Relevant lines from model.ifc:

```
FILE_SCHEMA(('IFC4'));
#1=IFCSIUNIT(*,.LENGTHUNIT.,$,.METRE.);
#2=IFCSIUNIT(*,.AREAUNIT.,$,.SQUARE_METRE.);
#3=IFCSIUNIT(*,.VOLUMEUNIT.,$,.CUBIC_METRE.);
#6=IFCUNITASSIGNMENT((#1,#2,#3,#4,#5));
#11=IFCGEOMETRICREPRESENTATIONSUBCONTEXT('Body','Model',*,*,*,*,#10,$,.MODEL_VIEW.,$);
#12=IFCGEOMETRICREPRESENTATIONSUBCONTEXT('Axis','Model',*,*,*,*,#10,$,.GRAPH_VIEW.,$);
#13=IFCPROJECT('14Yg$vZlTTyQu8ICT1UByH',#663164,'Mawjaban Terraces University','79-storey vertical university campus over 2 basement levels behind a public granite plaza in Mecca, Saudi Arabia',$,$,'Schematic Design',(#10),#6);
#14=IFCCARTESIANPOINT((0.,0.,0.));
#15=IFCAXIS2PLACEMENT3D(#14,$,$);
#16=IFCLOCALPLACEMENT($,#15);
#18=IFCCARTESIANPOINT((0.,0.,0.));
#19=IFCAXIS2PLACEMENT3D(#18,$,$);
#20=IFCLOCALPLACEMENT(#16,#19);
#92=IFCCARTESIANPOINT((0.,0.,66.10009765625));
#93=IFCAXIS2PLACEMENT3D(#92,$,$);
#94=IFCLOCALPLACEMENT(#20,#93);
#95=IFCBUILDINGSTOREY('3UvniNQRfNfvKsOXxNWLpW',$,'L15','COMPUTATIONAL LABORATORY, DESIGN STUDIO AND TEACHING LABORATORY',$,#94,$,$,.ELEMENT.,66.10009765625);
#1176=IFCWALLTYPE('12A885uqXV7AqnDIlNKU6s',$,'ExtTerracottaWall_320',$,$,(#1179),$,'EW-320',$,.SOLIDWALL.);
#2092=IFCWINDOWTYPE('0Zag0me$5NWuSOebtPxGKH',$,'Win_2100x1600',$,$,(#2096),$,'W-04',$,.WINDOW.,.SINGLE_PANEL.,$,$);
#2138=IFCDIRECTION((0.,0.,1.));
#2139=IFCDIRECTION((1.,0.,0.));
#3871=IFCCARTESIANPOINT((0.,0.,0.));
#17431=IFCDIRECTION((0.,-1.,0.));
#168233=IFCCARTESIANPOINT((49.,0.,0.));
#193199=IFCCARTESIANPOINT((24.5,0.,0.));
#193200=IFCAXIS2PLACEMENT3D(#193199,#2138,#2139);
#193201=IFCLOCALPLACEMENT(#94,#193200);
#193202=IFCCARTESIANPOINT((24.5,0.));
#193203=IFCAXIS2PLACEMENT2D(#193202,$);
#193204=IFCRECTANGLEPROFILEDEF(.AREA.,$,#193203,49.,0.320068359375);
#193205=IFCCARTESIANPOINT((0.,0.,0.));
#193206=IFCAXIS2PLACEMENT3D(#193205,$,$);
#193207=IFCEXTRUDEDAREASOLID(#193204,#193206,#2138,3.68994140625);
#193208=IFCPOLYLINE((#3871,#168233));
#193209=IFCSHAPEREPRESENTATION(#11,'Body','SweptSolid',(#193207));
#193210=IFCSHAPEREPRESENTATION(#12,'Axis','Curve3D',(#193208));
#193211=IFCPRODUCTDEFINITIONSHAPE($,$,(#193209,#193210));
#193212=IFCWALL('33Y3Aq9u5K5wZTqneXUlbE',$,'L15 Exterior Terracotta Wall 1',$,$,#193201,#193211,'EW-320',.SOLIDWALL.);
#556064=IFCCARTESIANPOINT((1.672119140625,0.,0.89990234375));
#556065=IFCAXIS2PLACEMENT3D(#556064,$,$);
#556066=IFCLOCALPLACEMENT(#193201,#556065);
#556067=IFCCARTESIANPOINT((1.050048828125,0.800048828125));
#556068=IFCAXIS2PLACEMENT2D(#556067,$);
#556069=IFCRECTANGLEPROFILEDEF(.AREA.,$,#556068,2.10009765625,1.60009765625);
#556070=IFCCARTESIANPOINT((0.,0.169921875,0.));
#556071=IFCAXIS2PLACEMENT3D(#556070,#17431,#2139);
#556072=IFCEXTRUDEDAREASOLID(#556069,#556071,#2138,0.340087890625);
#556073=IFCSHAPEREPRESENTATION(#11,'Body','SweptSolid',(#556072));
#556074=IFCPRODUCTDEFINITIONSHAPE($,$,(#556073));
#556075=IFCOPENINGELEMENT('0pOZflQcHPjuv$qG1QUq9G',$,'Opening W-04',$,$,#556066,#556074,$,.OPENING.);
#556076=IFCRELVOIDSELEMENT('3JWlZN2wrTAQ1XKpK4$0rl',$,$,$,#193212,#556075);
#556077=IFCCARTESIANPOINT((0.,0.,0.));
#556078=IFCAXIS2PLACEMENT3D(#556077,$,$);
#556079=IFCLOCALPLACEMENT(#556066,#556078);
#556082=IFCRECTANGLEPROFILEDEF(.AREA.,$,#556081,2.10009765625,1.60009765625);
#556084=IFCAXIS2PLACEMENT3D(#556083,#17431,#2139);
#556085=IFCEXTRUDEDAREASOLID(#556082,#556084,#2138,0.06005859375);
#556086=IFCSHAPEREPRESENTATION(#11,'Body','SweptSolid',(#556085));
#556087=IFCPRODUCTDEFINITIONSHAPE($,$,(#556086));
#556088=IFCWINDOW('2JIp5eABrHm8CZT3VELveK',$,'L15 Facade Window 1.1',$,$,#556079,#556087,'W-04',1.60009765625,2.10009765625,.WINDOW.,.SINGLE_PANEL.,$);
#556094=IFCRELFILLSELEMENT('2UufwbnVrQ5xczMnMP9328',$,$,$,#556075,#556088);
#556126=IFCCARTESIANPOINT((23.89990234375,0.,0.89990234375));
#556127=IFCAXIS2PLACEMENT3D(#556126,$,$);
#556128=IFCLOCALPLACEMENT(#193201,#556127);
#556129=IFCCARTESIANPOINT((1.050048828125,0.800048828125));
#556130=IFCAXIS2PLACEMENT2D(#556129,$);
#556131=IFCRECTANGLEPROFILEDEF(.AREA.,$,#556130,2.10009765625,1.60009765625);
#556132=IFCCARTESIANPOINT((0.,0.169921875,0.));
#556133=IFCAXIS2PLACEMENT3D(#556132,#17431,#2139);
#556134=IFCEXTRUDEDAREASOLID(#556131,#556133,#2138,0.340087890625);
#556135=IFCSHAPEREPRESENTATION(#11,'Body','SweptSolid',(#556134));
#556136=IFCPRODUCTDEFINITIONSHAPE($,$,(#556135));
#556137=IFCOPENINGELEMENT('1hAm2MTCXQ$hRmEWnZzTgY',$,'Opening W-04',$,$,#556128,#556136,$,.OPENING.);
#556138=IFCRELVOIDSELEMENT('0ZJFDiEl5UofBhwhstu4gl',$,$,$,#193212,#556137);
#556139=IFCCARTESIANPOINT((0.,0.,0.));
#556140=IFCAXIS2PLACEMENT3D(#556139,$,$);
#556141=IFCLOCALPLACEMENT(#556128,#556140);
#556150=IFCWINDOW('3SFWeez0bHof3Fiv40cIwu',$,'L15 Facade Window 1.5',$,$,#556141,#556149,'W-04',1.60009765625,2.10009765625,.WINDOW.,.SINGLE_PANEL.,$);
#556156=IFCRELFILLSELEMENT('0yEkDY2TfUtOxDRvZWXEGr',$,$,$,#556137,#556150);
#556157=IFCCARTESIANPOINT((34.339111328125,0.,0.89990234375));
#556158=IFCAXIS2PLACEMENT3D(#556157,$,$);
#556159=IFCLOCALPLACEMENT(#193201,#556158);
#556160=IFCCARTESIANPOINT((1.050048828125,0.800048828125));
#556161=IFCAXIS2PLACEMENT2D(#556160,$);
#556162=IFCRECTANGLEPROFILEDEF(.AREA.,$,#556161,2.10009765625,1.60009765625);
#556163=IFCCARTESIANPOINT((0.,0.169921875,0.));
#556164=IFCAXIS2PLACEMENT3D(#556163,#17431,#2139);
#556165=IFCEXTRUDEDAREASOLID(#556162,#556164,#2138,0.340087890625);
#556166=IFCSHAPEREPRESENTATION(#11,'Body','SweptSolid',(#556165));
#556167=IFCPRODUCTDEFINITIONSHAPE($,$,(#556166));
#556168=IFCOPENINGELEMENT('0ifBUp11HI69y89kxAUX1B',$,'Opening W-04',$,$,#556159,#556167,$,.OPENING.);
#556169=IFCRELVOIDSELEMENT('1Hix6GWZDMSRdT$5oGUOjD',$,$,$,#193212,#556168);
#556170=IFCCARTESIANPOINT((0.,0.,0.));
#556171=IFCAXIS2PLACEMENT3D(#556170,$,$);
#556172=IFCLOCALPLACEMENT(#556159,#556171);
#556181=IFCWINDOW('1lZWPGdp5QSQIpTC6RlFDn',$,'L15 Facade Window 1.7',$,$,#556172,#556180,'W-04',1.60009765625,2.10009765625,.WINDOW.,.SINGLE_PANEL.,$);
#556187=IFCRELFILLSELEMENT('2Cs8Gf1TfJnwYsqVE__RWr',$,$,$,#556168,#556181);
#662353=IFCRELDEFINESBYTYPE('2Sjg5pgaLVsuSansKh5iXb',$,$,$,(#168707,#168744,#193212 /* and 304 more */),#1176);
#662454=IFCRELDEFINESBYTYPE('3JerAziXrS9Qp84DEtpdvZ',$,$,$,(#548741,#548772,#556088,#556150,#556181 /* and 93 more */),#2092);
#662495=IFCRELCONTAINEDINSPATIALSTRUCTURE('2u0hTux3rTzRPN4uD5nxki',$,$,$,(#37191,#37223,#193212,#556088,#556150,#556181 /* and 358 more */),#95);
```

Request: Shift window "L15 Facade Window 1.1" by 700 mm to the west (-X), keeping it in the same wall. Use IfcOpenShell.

```python
import ifcopenshell
import ifcopenshell.api.geometry
import ifcopenshell.util.placement
import ifcopenshell.util.unit

model = ifcopenshell.open("model.ifc")
unit_scale = ifcopenshell.util.unit.calculate_unit_scale(model)

window = model.by_guid("2JIp5eABrHm8CZT3VELveK")
opening = window.FillsVoids[0].RelatingOpeningElement
wall = opening.VoidsElements[0].RelatingBuildingElement

wall_matrix = ifcopenshell.util.placement.get_local_placement(wall.ObjectPlacement)
shift = wall_matrix[:3, 0] * -0.7 / unit_scale
before = ifcopenshell.util.placement.get_local_placement(window.ObjectPlacement)[:3, 3].copy()

# The window is placed relative to its opening, so it follows when the opening moves.
matrix = ifcopenshell.util.placement.get_local_placement(opening.ObjectPlacement)
matrix[:3, 3] += shift
ifcopenshell.api.geometry.edit_object_placement(
    model, product=opening, matrix=matrix, is_si=False, should_transform_children=True
)

after = ifcopenshell.util.placement.get_local_placement(window.ObjectPlacement)[:3, 3]
print("window moved by", (after - before).round(3) + 0.0)

model.write("model_edited.ifc")
```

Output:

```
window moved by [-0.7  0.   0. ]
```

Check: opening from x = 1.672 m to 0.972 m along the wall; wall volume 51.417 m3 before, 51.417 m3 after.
